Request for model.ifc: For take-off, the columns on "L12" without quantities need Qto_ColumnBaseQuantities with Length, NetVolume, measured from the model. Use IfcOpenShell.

First a look at what the model holds.

```python
import ifcopenshell
import ifcopenshell.util.element
import ifcopenshell.util.unit

model = ifcopenshell.open("model.ifc")
print(model.schema)
for unit_type in ("LENGTHUNIT", "AREAUNIT", "VOLUMEUNIT"):
    print(unit_type, ifcopenshell.util.unit.calculate_unit_scale(model, unit_type))
storey = next(s for s in model.by_type("IfcBuildingStorey") if s.Name == "L12")
columns = [e for e in ifcopenshell.util.element.get_decomposition(storey) if e.is_a("IfcColumn")]
for e in sorted(columns, key=lambda e: e.id()):
    print(e.id(), e.is_a(), e.Name, list(ifcopenshell.util.element.get_psets(e, qtos_only=True)), sep=" | ")
```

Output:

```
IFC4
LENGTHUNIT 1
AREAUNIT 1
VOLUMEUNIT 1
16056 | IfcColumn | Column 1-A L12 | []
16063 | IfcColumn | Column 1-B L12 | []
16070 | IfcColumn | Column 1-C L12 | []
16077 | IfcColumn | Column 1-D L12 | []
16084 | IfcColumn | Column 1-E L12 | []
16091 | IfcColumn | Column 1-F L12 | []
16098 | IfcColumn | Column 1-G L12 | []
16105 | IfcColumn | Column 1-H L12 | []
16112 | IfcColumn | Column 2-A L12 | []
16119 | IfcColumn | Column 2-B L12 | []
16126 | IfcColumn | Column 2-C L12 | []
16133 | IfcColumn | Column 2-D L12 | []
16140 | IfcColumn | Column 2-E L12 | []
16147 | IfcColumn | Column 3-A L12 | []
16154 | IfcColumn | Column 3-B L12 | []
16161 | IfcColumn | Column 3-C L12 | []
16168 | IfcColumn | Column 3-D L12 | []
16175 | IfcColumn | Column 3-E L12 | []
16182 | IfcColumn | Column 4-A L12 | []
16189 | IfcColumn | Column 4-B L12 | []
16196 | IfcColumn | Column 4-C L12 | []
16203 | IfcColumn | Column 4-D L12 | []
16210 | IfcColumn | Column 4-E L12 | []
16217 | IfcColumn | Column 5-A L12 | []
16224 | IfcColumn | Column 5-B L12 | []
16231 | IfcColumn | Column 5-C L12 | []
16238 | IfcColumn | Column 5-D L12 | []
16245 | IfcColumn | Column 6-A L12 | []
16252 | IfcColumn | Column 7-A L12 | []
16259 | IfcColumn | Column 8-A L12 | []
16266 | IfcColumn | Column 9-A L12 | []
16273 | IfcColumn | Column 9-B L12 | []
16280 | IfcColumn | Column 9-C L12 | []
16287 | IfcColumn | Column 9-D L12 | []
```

```python
import ifcopenshell
import ifcopenshell.api.pset
import ifcopenshell.geom
import ifcopenshell.util.element
import ifcopenshell.util.shape
import ifcopenshell.util.unit

model = ifcopenshell.open("model.ifc")
unit_scale = ifcopenshell.util.unit.calculate_unit_scale(model)
volume_scale = ifcopenshell.util.unit.calculate_unit_scale(model, "VOLUMEUNIT")
settings = ifcopenshell.geom.settings()

storey = next(s for s in model.by_type("IfcBuildingStorey") if s.Name == "L12")
columns = [e for e in ifcopenshell.util.element.get_decomposition(storey) if e.is_a("IfcColumn")]

for e in sorted(columns, key=lambda e: e.id()):
    if ifcopenshell.util.element.get_psets(e, qtos_only=True, should_inherit=False):
        continue
    # Geometry comes back in metres, in the element's own axes.
    shape = ifcopenshell.geom.create_shape(settings, e)
    values = {
        "Length": ifcopenshell.util.shape.get_z(shape.geometry) / unit_scale,
        "NetVolume": ifcopenshell.util.shape.get_volume(shape.geometry) / volume_scale,
    }
    qto = ifcopenshell.api.pset.add_qto(model, product=e, name="Qto_ColumnBaseQuantities")
    ifcopenshell.api.pset.edit_qto(model, qto=qto, properties=values)
    print(e.id(), {k: round(v, 3) for k, v in values.items()})

model.write("model_edited.ifc")
```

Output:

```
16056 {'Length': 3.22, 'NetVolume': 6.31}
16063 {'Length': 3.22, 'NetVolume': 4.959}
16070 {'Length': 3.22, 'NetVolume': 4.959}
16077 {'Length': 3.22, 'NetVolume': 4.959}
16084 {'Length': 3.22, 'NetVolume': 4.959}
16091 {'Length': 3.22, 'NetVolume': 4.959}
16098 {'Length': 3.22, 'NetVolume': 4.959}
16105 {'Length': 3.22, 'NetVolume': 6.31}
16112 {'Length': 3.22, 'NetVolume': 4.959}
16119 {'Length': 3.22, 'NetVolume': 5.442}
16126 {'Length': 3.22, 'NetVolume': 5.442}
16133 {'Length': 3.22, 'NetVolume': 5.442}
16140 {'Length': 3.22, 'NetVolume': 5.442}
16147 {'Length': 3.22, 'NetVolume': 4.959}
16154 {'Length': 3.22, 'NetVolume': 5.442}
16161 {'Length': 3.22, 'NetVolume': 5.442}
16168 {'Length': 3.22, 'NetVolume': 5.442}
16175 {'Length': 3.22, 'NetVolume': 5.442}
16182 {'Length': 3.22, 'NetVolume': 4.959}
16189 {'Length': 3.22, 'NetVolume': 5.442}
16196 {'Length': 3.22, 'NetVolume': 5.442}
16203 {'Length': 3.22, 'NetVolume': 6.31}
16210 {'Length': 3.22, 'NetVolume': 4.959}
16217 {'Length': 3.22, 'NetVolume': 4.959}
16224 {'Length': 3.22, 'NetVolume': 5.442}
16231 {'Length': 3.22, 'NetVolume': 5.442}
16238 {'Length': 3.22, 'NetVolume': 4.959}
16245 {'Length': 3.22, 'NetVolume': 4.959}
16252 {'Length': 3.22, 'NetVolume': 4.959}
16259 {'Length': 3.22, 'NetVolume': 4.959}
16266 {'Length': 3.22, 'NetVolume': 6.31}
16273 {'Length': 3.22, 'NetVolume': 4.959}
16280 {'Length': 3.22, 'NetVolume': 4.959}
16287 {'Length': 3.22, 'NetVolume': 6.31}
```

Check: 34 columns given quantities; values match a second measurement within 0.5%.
